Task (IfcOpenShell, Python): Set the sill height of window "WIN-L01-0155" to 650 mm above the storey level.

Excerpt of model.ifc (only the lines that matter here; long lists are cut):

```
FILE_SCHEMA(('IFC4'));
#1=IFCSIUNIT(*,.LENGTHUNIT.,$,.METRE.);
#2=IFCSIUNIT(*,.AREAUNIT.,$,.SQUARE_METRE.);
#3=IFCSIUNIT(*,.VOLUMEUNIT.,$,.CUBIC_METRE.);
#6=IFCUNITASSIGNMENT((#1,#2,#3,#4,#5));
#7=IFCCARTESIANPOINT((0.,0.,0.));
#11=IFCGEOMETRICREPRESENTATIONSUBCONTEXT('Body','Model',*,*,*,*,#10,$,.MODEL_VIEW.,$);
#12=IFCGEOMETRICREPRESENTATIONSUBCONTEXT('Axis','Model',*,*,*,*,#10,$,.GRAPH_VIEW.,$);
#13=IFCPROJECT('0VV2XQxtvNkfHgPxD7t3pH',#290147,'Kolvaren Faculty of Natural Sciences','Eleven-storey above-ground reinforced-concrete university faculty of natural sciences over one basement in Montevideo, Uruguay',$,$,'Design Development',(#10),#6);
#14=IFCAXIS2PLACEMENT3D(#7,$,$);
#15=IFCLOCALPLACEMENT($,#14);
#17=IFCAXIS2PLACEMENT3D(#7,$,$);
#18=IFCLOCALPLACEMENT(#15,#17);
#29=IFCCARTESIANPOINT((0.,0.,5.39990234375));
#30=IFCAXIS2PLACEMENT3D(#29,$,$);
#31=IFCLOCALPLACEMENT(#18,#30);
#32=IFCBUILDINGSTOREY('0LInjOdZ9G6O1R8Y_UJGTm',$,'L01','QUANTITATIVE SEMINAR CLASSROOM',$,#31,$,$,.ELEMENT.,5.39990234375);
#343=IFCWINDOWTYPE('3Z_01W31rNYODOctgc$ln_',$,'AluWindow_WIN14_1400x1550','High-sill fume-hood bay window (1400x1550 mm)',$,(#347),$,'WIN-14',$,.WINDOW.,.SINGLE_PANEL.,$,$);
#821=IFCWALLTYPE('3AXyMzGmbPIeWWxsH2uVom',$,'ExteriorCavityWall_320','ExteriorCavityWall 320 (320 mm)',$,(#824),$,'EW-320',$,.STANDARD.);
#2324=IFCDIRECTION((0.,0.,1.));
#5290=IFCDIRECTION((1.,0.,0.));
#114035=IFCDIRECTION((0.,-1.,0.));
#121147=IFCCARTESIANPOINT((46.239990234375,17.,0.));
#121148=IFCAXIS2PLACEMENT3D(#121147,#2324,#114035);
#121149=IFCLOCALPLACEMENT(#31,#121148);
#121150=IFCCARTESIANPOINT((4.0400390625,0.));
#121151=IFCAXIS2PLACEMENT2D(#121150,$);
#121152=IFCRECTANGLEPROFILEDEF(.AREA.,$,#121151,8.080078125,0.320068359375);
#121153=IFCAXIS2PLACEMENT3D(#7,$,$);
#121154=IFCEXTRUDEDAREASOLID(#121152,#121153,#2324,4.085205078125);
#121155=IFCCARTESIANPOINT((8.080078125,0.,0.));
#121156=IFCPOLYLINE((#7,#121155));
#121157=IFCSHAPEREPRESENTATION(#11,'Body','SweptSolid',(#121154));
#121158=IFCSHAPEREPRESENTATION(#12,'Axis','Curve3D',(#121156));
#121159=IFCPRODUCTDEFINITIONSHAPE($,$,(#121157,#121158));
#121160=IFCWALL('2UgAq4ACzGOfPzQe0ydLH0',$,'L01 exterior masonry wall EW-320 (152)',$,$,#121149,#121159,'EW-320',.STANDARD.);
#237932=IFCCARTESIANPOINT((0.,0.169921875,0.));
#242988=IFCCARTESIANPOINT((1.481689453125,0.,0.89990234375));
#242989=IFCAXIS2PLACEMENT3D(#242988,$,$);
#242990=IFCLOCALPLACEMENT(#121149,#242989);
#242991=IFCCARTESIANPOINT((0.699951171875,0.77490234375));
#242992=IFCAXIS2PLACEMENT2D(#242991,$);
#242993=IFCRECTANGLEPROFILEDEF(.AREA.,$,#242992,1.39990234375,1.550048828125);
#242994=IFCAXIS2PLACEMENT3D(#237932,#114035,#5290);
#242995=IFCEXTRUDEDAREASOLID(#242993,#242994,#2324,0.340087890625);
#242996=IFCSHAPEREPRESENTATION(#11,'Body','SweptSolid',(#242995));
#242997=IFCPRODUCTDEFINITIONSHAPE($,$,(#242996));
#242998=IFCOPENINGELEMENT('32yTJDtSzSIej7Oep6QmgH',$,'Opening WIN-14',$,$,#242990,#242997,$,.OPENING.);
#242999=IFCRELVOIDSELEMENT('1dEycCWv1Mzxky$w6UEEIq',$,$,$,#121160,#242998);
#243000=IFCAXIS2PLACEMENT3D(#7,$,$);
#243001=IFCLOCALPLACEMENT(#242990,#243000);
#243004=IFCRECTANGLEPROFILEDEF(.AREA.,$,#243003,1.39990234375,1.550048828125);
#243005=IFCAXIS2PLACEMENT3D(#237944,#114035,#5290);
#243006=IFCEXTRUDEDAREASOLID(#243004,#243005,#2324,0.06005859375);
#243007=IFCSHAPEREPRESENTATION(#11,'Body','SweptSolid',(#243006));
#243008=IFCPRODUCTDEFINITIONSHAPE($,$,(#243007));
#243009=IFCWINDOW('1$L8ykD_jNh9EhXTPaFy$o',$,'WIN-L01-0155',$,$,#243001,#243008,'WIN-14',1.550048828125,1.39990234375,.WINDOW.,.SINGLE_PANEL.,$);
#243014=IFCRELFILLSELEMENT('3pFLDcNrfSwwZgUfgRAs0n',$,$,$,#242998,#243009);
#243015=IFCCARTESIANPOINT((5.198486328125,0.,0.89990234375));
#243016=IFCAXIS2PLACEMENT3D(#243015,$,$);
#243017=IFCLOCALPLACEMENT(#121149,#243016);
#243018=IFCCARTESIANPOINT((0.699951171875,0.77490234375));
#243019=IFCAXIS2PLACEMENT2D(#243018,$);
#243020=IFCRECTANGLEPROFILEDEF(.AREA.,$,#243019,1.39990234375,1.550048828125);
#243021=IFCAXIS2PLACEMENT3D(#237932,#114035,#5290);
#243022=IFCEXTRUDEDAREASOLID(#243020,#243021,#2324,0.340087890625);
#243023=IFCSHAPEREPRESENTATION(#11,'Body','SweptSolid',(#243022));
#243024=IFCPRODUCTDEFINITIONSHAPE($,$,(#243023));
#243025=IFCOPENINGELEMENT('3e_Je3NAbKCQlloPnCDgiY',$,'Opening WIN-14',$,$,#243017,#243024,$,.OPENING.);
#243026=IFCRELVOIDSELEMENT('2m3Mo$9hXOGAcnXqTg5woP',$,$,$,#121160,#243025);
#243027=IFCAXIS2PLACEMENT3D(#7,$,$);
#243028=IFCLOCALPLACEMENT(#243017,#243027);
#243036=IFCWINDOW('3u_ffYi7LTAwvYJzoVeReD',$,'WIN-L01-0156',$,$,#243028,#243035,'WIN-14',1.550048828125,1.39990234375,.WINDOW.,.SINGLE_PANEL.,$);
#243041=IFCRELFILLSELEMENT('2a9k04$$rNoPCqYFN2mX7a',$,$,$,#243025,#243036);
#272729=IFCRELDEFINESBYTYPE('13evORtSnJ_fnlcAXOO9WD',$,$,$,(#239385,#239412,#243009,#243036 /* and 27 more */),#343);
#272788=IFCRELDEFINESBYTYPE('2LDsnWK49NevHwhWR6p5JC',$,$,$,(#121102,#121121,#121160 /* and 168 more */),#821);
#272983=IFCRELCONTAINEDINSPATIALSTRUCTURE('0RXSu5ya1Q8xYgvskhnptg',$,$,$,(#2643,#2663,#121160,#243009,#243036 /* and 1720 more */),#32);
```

```python
import numpy as np
import ifcopenshell
import ifcopenshell.api.geometry
import ifcopenshell.geom
import ifcopenshell.util.element
import ifcopenshell.util.placement
import ifcopenshell.util.shape
import ifcopenshell.util.unit

model = ifcopenshell.open("model.ifc")
unit_scale = ifcopenshell.util.unit.calculate_unit_scale(model)

window = model.by_id(243009)
opening = window.FillsVoids[0].RelatingOpeningElement
storey = ifcopenshell.util.element.get_container(window, ifc_class="IfcBuildingStorey")
level = ifcopenshell.util.placement.get_local_placement(storey.ObjectPlacement)[2, 3]

# The opening's origin need not be at the sill, so measure its lowest point.
shape = ifcopenshell.geom.create_shape(ifcopenshell.geom.settings(), opening)
bottom = ifcopenshell.util.shape.get_shape_bottom_elevation(shape, shape.geometry) / unit_scale
dz = level + 0.65 / unit_scale - bottom

shift = np.array([0.0, 0.0, dz])
# The window is placed relative to its opening, so it follows when the opening moves.
matrix = ifcopenshell.util.placement.get_local_placement(opening.ObjectPlacement)
matrix[:3, 3] += shift
ifcopenshell.api.geometry.edit_object_placement(
    model, product=opening, matrix=matrix, is_si=False, should_transform_children=True
)

print(f"moved by {dz * unit_scale:+.3f} m")

model.write("model_v2.ifc")
```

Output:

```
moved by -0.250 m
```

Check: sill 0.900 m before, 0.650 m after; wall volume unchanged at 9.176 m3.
